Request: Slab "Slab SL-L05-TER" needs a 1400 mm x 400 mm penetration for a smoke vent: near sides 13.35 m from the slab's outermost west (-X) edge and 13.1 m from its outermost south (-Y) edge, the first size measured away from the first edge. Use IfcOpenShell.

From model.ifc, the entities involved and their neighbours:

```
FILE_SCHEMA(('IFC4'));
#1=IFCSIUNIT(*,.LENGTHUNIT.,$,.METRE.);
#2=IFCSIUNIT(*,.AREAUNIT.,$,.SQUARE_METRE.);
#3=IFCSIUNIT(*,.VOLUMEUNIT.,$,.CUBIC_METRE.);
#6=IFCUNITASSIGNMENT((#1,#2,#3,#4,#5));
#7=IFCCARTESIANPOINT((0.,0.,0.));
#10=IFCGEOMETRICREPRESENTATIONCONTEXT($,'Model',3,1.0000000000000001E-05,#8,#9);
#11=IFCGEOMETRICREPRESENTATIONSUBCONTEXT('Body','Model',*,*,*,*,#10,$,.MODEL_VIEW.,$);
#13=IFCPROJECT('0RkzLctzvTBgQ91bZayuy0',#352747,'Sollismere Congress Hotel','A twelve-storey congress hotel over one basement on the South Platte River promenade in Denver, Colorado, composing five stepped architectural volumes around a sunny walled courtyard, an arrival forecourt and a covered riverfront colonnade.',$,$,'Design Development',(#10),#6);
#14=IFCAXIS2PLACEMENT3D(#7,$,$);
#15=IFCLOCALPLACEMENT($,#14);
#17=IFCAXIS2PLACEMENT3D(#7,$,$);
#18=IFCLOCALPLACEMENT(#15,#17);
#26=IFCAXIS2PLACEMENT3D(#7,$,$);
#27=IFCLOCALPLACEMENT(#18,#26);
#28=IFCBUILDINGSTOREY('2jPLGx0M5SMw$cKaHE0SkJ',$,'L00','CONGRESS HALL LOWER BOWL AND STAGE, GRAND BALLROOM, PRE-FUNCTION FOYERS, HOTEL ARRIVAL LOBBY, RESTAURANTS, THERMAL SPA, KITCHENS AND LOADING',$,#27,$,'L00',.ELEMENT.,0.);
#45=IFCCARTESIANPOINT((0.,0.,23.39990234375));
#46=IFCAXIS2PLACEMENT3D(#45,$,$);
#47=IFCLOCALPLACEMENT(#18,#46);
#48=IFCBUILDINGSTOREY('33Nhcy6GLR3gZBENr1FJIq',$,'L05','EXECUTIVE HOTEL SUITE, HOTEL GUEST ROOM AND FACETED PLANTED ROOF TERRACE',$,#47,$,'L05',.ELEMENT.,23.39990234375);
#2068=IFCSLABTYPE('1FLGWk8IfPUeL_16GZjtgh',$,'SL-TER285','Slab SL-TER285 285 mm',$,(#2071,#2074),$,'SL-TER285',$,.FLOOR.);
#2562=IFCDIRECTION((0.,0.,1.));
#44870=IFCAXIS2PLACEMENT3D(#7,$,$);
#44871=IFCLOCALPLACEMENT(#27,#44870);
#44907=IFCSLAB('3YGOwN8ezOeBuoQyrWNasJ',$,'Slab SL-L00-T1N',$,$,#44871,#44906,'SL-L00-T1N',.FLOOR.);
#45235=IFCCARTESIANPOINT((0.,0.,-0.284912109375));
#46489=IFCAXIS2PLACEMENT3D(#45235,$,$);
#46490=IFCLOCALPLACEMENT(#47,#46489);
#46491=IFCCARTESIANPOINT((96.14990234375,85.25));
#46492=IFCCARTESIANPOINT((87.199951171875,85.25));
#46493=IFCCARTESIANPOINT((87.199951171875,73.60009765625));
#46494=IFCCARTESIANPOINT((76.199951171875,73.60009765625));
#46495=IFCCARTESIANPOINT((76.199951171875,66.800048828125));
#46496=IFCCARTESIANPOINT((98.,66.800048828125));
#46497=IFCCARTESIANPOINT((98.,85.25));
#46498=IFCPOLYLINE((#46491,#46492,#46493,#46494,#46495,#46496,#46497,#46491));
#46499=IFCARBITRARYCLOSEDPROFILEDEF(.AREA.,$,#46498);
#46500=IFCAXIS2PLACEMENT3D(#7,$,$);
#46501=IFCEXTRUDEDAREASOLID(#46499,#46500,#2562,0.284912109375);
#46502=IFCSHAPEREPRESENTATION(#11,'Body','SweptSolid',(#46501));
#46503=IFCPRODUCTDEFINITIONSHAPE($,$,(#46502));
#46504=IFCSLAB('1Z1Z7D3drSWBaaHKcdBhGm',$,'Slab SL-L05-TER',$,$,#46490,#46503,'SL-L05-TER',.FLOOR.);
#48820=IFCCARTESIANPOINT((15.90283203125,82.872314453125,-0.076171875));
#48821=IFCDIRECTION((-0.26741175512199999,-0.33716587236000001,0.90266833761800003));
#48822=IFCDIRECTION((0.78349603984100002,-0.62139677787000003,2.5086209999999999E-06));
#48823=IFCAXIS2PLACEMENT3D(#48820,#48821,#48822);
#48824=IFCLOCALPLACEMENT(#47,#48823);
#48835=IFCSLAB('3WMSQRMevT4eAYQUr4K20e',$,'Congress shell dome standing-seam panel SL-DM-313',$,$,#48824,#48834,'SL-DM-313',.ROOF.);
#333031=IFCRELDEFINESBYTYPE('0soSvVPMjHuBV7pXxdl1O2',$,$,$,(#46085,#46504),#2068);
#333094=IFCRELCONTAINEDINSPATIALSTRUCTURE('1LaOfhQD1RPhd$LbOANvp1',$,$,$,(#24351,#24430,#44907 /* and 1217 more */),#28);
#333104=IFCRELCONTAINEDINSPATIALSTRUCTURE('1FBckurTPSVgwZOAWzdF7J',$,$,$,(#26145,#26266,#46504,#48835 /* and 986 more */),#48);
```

```python
import numpy as np
import ifcopenshell
import ifcopenshell.api.feature
import ifcopenshell.api.geometry
import ifcopenshell.api.root
import ifcopenshell.geom
import ifcopenshell.util.placement
import ifcopenshell.util.representation
import ifcopenshell.util.shape
import ifcopenshell.util.unit

model = ifcopenshell.open("model.ifc")
unit_scale = ifcopenshell.util.unit.calculate_unit_scale(model)
settings = ifcopenshell.geom.settings()


def volume(element):
    """Net volume in cubic metres, openings subtracted."""
    shape = ifcopenshell.geom.create_shape(settings, element)
    return ifcopenshell.util.shape.get_volume(shape.geometry)


slab = model.by_guid("1Z1Z7D3drSWBaaHKcdBhGm")
before = volume(slab)

# Extent in the slab's own axes, in metres. The edges named are its -X and -Y sides.
slab_shape = ifcopenshell.geom.create_shape(settings, slab)
vertices = ifcopenshell.util.shape.get_vertices(slab_shape.geometry)
x_min, y_min, bottom = vertices.min(axis=0)
top = vertices[:, 2].max()

opening = ifcopenshell.api.root.create_entity(model, ifc_class="IfcOpeningElement", name="Smoke vent opening", predefined_type="OPENING")
context = ifcopenshell.util.representation.get_context(model, "Model", "Body", "MODEL_VIEW")
width, depth = 1.4, 0.4
outline = [(0.0, 0.0), (width, 0.0), (width, depth), (0.0, depth), (0.0, 0.0)]
# Overshoot both faces by 50 mm so the cut is clean.
shape = ifcopenshell.api.geometry.add_slab_representation(
    model, context=context, depth=top - bottom + 0.1, polyline=outline
)
ifcopenshell.api.geometry.assign_representation(model, product=opening, representation=shape)

matrix = ifcopenshell.util.placement.get_local_placement(slab.ObjectPlacement)
matrix[:, 3] = matrix @ np.append(np.array([x_min + 13.35, y_min + 13.1, bottom - 0.05]) / unit_scale, 1.0)
ifcopenshell.api.geometry.edit_object_placement(model, product=opening, matrix=matrix, is_si=False)
ifcopenshell.api.feature.add_feature(model, feature=opening, element=slab)

after = volume(slab)

print(f"slab volume {before:.3f} -> {after:.3f} m3")

model.write("model_updated.ifc")
```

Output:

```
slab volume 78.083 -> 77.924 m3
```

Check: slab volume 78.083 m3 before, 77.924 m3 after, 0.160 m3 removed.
